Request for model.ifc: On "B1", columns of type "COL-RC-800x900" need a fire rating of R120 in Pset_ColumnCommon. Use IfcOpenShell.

First a look at what the model holds.

```python
import ifcopenshell
import ifcopenshell.util.element

model = ifcopenshell.open("model.ifc")
print(model.schema)
storey = next(s for s in model.by_type("IfcBuildingStorey") if s.Name == "B1")
columns = [e for e in ifcopenshell.util.element.get_decomposition(storey) if e.is_a("IfcColumn")]
seen = {}
for e in columns:
    element_type = ifcopenshell.util.element.get_type(e)
    key = (element_type.Name if element_type != e and element_type else None, ifcopenshell.util.element.get_pset(e, "Pset_ColumnCommon", "FireRating"))
    seen[key] = seen.get(key, 0) + 1
for (name, value), count in sorted(seen.items(), key=str):
    print(count, "x", name, "|", value)
```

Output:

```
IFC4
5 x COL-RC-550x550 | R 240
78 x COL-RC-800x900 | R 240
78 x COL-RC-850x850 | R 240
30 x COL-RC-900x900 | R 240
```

```python
import ifcopenshell
import ifcopenshell.api.pset
import ifcopenshell.util.element

model = ifcopenshell.open("model.ifc")

storey = next(s for s in model.by_type("IfcBuildingStorey") if s.Name == "B1")
columns = [e for e in ifcopenshell.util.element.get_decomposition(storey) if e.is_a("IfcColumn")]

count = 0
for e in columns:
    element_type = ifcopenshell.util.element.get_type(e)
    if element_type in (None, e) or element_type.Name != "COL-RC-800x900":
        continue
    # add_pset returns the element's existing set when there is one.
    pset = ifcopenshell.api.pset.add_pset(model, product=e, name="Pset_ColumnCommon")
    ifcopenshell.api.pset.edit_pset(model, pset=pset, properties={"FireRating": "R120"})
    count += 1

print(count, "columns updated")

model.write("model_rev.ifc")
```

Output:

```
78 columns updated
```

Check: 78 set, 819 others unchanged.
